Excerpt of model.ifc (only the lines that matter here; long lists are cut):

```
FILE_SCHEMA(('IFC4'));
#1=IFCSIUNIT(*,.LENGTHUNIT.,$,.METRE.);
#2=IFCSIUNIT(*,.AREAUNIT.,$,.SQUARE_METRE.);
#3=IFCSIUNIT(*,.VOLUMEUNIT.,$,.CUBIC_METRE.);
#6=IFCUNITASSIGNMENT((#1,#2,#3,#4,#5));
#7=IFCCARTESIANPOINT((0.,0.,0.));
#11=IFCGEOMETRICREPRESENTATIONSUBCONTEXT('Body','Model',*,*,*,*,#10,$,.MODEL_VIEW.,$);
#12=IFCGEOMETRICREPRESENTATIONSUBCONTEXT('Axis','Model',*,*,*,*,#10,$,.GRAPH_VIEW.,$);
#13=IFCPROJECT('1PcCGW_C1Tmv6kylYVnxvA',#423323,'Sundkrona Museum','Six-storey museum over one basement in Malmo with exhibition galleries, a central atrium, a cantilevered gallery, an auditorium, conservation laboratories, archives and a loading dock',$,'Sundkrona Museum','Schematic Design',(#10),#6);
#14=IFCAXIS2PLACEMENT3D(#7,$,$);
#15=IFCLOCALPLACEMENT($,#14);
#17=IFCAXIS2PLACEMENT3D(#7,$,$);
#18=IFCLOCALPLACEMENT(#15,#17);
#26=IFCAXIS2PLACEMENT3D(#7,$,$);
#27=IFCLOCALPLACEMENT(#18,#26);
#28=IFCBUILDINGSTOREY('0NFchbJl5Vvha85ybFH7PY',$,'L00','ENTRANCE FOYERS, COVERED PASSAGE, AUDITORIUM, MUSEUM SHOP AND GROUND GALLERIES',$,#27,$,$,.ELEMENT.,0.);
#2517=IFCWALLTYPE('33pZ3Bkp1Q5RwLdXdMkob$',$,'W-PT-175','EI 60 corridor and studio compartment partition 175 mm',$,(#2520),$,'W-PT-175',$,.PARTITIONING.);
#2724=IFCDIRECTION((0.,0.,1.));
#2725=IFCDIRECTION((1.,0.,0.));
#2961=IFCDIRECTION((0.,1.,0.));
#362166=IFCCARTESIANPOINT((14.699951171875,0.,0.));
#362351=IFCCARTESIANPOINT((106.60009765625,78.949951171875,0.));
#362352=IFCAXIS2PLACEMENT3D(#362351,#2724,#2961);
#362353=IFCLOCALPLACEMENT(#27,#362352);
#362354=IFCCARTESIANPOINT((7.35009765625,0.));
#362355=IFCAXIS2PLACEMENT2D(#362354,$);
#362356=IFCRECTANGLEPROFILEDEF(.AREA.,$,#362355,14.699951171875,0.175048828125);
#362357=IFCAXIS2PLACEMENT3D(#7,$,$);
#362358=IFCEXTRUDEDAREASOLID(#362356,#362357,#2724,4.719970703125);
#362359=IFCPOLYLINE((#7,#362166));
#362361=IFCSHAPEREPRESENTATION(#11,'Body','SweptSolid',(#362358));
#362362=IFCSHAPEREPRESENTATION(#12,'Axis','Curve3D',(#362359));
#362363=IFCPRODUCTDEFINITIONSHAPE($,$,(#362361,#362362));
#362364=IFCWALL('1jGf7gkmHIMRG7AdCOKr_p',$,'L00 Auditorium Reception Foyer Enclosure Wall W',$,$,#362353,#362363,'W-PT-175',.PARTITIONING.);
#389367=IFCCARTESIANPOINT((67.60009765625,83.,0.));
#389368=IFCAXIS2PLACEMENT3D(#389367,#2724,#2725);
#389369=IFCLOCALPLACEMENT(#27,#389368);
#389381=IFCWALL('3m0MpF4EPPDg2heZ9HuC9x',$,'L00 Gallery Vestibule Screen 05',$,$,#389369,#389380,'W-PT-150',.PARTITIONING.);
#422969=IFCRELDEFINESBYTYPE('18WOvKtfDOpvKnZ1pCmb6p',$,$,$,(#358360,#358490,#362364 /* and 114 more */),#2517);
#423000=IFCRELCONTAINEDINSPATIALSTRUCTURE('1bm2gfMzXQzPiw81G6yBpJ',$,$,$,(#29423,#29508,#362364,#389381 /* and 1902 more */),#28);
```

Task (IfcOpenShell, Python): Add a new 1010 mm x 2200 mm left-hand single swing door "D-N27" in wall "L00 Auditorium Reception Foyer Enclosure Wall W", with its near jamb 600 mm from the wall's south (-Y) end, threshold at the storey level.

```python
import numpy as np
import ifcopenshell
import ifcopenshell.api.feature
import ifcopenshell.api.geometry
import ifcopenshell.api.root
import ifcopenshell.api.spatial
import ifcopenshell.geom
import ifcopenshell.util.element
import ifcopenshell.util.placement
import ifcopenshell.util.representation
import ifcopenshell.util.shape
import ifcopenshell.util.unit

model = ifcopenshell.open("model.ifc")
unit_scale = ifcopenshell.util.unit.calculate_unit_scale(model)
settings = ifcopenshell.geom.settings()


def volume(element):
    """Net volume in cubic metres, openings subtracted."""
    shape = ifcopenshell.geom.create_shape(settings, element)
    return ifcopenshell.util.shape.get_volume(shape.geometry)


wall = model.by_guid("1jGf7gkmHIMRG7AdCOKr_p")
storey = ifcopenshell.util.element.get_container(wall, ifc_class="IfcBuildingStorey")
context = ifcopenshell.util.representation.get_context(model, "Model", "Body", "MODEL_VIEW")
before = volume(wall)

width, height, from_end, sill = 1.01, 2.2, 0.6, 0.0  # metres

# The wall runs along its own X axis, and the end named is its -X end.
wall_shape = ifcopenshell.geom.create_shape(settings, wall)
x, y, z = ifcopenshell.util.shape.get_vertices(wall_shape.geometry).T
start = x.min() + from_end
face, thickness = float(y.min()), float(y.max() - y.min())
wall_matrix = ifcopenshell.util.placement.get_local_placement(wall.ObjectPlacement)
level = ifcopenshell.util.placement.get_local_placement(storey.ObjectPlacement)[2, 3]


def in_wall(x, y):
    """Placement at x, y metres in the wall's axes, at sill height."""
    matrix = wall_matrix.copy()
    matrix[:, 3] = wall_matrix @ np.array([x / unit_scale, y / unit_scale, 0.0, 1.0])
    matrix[2, 3] = level + sill / unit_scale
    return matrix


# Opening: a box that overshoots both wall faces by 50 mm.
opening = ifcopenshell.api.root.create_entity(model, ifc_class="IfcOpeningElement", predefined_type="OPENING")
box = ifcopenshell.api.geometry.add_wall_representation(
    model, context=context, length=width, height=height, thickness=thickness + 0.1
)
ifcopenshell.api.geometry.assign_representation(model, product=opening, representation=box)
ifcopenshell.api.geometry.edit_object_placement(model, product=opening, matrix=in_wall(start, face - 0.05), is_si=False)
ifcopenshell.api.feature.add_feature(model, feature=opening, element=wall)

door = ifcopenshell.api.root.create_entity(model, ifc_class="IfcDoor", name="D-N27", predefined_type="DOOR")
door.OverallWidth, door.OverallHeight = width / unit_scale, height / unit_scale
door.OperationType = "SINGLE_SWING_LEFT"
body = ifcopenshell.api.geometry.add_door_representation(
    model,
    context=context,
    overall_width=door.OverallWidth,
    overall_height=door.OverallHeight,
    operation_type="SINGLE_SWING_LEFT",
    lining_properties={"LiningDepth": thickness / unit_scale, "ThresholdDepth": thickness / unit_scale},
)
ifcopenshell.api.geometry.assign_representation(model, product=door, representation=body)
ifcopenshell.api.spatial.assign_container(model, products=[door], relating_structure=storey)
ifcopenshell.api.feature.add_filling(model, opening=opening, element=door)

# The lining spans the wall, so the door starts at the wall face.
ifcopenshell.api.geometry.edit_object_placement(model, product=door, matrix=in_wall(start, face), is_si=False)

after = volume(wall)

print(f"wall volume {before:.3f} -> {after:.3f} m3")

model.write("model_rev.ifc")
```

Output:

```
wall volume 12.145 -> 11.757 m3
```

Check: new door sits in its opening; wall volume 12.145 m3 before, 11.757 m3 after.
